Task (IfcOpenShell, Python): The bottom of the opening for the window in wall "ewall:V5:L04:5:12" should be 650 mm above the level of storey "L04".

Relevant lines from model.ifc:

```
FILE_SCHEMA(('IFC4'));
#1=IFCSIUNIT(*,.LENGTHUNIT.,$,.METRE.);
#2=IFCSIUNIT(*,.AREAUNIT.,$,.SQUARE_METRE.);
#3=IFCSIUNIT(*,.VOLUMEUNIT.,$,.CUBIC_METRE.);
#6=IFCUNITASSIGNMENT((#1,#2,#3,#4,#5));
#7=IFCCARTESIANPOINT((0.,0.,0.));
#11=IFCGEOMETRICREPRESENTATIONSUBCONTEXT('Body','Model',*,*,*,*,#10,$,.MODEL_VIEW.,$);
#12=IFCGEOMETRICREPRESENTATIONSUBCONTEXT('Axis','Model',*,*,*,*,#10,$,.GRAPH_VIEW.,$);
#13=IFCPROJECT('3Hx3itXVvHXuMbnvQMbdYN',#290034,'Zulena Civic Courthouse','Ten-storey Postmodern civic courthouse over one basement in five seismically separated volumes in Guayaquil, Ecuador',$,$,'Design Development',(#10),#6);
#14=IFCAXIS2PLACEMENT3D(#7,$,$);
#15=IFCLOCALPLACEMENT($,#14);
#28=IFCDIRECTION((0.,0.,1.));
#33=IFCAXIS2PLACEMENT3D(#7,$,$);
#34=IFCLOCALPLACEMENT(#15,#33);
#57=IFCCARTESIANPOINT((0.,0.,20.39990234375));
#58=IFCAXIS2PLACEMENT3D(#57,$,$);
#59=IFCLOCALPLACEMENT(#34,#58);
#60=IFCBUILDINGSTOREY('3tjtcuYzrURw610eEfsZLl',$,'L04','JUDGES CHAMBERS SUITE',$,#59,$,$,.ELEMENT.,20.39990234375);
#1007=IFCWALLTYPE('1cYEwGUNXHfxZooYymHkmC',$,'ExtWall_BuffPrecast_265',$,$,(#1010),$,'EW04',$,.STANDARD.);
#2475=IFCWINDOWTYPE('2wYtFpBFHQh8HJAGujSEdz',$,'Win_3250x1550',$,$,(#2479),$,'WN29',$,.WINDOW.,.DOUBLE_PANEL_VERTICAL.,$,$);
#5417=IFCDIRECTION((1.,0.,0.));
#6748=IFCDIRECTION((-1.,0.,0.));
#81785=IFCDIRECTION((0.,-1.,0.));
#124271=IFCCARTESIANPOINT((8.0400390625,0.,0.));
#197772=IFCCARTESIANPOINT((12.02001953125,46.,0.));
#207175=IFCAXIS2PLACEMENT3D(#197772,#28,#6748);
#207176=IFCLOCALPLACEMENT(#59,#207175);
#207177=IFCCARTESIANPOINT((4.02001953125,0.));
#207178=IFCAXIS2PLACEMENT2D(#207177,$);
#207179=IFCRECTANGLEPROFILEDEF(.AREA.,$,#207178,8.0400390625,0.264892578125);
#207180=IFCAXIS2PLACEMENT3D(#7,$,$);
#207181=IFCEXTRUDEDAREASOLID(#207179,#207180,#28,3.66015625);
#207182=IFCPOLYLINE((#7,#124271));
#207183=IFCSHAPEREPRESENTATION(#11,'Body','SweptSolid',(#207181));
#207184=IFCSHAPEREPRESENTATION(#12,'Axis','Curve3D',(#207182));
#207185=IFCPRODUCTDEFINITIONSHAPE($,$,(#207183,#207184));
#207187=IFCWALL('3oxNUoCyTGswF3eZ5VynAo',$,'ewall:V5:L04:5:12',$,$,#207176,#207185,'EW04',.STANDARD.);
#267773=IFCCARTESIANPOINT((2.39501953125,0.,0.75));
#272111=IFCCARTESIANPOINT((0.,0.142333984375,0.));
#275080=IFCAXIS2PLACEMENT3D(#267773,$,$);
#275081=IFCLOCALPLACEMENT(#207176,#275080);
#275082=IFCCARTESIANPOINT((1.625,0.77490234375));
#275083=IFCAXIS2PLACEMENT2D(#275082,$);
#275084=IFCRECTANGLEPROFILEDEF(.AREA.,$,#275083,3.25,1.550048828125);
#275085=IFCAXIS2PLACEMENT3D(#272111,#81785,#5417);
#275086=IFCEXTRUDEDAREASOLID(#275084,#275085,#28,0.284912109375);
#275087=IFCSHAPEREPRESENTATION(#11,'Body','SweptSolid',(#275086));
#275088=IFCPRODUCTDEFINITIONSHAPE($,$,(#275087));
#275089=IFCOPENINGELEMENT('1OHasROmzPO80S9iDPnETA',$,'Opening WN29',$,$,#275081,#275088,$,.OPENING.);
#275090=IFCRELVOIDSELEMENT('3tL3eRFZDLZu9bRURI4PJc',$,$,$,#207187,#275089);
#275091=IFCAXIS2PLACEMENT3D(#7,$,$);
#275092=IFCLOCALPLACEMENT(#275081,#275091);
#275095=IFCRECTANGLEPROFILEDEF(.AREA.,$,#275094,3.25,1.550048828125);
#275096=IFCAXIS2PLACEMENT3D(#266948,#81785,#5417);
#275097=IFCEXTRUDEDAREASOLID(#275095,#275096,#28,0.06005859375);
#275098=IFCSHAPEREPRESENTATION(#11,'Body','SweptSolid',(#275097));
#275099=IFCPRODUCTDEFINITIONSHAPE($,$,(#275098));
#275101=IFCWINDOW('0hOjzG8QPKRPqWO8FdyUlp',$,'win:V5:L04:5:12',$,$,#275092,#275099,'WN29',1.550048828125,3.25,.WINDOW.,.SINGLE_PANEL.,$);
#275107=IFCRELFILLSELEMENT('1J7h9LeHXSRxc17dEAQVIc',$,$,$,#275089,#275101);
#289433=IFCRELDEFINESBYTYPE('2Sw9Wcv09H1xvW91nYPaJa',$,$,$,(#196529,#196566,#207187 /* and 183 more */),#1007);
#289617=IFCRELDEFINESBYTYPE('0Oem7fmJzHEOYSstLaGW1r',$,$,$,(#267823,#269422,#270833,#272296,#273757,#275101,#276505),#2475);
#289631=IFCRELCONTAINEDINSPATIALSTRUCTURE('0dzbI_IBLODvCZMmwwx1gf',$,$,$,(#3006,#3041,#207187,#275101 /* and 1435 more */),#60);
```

```python
import numpy as np
import ifcopenshell
import ifcopenshell.api.geometry
import ifcopenshell.geom
import ifcopenshell.util.element
import ifcopenshell.util.placement
import ifcopenshell.util.shape
import ifcopenshell.util.unit

model = ifcopenshell.open("model.ifc")
unit_scale = ifcopenshell.util.unit.calculate_unit_scale(model)

window = model.by_guid("0hOjzG8QPKRPqWO8FdyUlp")
opening = window.FillsVoids[0].RelatingOpeningElement
storey = ifcopenshell.util.element.get_container(window, ifc_class="IfcBuildingStorey")
level = ifcopenshell.util.placement.get_local_placement(storey.ObjectPlacement)[2, 3]

# The opening's origin need not be at the sill, so measure its lowest point.
shape = ifcopenshell.geom.create_shape(ifcopenshell.geom.settings(), opening)
bottom = ifcopenshell.util.shape.get_shape_bottom_elevation(shape, shape.geometry) / unit_scale
dz = level + 0.65 - bottom

shift = np.array([0.0, 0.0, dz])
# The window is placed relative to its opening, so it follows when the opening moves.
matrix = ifcopenshell.util.placement.get_local_placement(opening.ObjectPlacement)
matrix[:3, 3] += shift
ifcopenshell.api.geometry.edit_object_placement(
    model, product=opening, matrix=matrix, is_si=False, should_transform_children=True
)

print(f"moved by {dz * unit_scale:+.3f} m")

model.write("model_updated.ifc")
```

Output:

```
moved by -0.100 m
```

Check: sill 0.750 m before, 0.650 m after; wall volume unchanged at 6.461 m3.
